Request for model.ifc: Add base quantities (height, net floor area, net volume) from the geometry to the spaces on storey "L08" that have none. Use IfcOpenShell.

First a look at what the model holds.

```python
import ifcopenshell
import ifcopenshell.util.element
import ifcopenshell.util.unit

model = ifcopenshell.open("model.ifc")
print(model.schema)
for unit_type in ("LENGTHUNIT", "AREAUNIT", "VOLUMEUNIT"):
    print(unit_type, ifcopenshell.util.unit.calculate_unit_scale(model, unit_type))
storey = next(s for s in model.by_type("IfcBuildingStorey") if s.Name == "L08")
spaces = [e for e in ifcopenshell.util.element.get_decomposition(storey) if e.is_a("IfcSpace")]
for e in sorted(spaces, key=lambda e: e.id()):
    print(e.id(), e.is_a(), e.Name, list(ifcopenshell.util.element.get_psets(e, qtos_only=True)), sep=" | ")
```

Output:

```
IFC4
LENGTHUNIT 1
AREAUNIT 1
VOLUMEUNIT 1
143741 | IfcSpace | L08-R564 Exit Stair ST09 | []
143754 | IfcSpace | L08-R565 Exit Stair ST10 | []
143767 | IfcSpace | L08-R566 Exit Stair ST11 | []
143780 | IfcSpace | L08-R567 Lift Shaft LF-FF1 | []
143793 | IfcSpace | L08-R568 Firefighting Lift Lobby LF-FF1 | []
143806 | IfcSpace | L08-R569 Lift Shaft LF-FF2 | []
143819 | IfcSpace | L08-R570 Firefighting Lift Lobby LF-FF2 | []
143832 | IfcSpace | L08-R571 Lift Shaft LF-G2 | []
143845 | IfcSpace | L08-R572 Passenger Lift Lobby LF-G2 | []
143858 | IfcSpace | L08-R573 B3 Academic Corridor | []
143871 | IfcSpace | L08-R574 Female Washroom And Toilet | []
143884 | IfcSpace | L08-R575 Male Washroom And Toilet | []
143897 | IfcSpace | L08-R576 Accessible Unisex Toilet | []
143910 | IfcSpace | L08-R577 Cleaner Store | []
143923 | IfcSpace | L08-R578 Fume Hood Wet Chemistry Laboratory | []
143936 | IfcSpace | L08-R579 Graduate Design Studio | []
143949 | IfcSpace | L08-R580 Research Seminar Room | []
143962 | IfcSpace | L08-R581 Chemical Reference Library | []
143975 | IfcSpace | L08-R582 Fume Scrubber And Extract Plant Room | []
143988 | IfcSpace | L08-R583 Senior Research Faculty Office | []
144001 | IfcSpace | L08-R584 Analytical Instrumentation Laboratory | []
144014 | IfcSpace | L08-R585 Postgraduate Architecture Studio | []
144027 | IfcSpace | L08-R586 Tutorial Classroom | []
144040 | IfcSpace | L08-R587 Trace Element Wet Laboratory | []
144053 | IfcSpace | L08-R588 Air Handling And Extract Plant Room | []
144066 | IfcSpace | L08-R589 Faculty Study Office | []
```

```python
import ifcopenshell
import ifcopenshell.api.pset
import ifcopenshell.geom
import ifcopenshell.util.element
import ifcopenshell.util.shape
import ifcopenshell.util.unit

model = ifcopenshell.open("model.ifc")
unit_scale = ifcopenshell.util.unit.calculate_unit_scale(model)
area_scale = ifcopenshell.util.unit.calculate_unit_scale(model, "AREAUNIT")
volume_scale = ifcopenshell.util.unit.calculate_unit_scale(model, "VOLUMEUNIT")
settings = ifcopenshell.geom.settings()

storey = next(s for s in model.by_type("IfcBuildingStorey") if s.Name == "L08")
spaces = [e for e in ifcopenshell.util.element.get_decomposition(storey) if e.is_a("IfcSpace")]

for e in sorted(spaces, key=lambda e: e.id()):
    if ifcopenshell.util.element.get_psets(e, qtos_only=True, should_inherit=False):
        continue
    # Geometry comes back in metres, in the element's own axes.
    shape = ifcopenshell.geom.create_shape(settings, e)
    values = {
        "Height": ifcopenshell.util.shape.get_z(shape.geometry) / unit_scale,
        "NetFloorArea": ifcopenshell.util.shape.get_footprint_area(shape.geometry) / area_scale,
        "NetVolume": ifcopenshell.util.shape.get_volume(shape.geometry) / volume_scale,
    }
    qto = ifcopenshell.api.pset.add_qto(model, product=e, name="Qto_SpaceBaseQuantities")
    ifcopenshell.api.pset.edit_qto(model, qto=qto, properties=values)
    print(e.id(), {k: round(v, 3) for k, v in values.items()})

model.write("model_v2.ifc")
```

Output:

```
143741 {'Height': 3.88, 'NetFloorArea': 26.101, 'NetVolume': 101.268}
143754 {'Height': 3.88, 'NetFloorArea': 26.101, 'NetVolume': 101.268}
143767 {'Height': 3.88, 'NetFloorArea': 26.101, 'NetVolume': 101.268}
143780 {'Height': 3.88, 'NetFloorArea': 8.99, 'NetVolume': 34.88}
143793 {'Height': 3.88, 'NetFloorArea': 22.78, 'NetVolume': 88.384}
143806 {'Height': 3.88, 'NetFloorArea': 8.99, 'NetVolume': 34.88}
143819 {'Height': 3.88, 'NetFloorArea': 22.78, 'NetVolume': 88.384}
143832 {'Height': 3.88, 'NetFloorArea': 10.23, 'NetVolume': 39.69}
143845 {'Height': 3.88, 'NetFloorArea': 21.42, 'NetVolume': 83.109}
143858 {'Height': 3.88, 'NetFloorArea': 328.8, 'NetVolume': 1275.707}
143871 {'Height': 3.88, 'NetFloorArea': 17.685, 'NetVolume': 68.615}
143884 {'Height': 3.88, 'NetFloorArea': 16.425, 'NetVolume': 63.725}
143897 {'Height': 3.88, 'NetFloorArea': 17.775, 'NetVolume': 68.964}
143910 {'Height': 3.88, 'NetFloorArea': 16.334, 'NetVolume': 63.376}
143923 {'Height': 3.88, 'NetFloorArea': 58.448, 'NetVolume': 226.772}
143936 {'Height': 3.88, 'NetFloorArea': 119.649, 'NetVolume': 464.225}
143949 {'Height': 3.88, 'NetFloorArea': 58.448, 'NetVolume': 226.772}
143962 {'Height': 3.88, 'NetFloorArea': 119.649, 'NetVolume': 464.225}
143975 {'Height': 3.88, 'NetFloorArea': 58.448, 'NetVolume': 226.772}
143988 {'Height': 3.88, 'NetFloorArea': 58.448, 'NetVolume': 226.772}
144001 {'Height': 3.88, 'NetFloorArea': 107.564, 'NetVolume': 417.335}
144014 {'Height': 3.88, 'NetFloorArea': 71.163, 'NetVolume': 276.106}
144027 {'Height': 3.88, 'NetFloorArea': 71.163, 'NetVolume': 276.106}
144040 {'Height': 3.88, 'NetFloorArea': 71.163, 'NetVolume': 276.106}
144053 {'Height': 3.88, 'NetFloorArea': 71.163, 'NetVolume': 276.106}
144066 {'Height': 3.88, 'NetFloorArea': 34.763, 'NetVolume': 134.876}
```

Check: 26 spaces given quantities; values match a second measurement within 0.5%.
